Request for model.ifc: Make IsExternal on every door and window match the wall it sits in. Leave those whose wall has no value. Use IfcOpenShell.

First a look at what the model holds.

```python
import ifcopenshell
import ifcopenshell.util.element

model = ifcopenshell.open("model.ifc")
print(model.schema)
seen = {}
for e in model.by_type("IfcDoor") + model.by_type("IfcWindow"):
    if not e.FillsVoids:
        continue
    host = e.FillsVoids[0].RelatingOpeningElement.VoidsElements[0].RelatingBuildingElement
    own = ifcopenshell.util.element.get_pset(e, f"Pset_{e.is_a()[3:].removesuffix('StandardCase')}Common", "IsExternal")
    wall = ifcopenshell.util.element.get_pset(host, "Pset_WallCommon", "IsExternal")
    seen[e.is_a(), own, wall] = seen.get((e.is_a(), own, wall), 0) + 1
for (cls, own, wall), count in sorted(seen.items(), key=str):
    print(count, cls, "IsExternal:", own, "| host wall:", wall)
```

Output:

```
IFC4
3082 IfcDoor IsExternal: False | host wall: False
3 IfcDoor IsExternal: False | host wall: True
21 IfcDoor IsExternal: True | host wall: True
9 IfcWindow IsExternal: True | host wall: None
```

```python
import ifcopenshell
import ifcopenshell.api.pset
import ifcopenshell.util.element

model = ifcopenshell.open("model.ifc")

count = 0
for ifc_class, pset_name in (("IfcDoor", "Pset_DoorCommon"), ("IfcWindow", "Pset_WindowCommon")):
    for e in model.by_type(ifc_class):
        if not e.FillsVoids:
            continue
        host = e.FillsVoids[0].RelatingOpeningElement.VoidsElements[0].RelatingBuildingElement
        external = ifcopenshell.util.element.get_pset(host, "Pset_WallCommon", "IsExternal")
        if external is None or ifcopenshell.util.element.get_pset(e, pset_name, "IsExternal") == external:
            continue
        pset = ifcopenshell.api.pset.add_pset(model, product=e, name=pset_name)
        ifcopenshell.api.pset.edit_pset(model, pset=pset, properties={"IsExternal": external})
        count += 1

print(count, "updated")

model.write("model_rev.ifc")
```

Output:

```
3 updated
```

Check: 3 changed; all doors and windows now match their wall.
